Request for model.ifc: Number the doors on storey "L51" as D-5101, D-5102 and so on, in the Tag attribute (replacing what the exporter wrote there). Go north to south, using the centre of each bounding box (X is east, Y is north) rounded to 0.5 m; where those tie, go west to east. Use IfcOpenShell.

First a look at what the model holds.

```python
import ifcopenshell
import ifcopenshell.util.element
import ifcopenshell.util.placement

model = ifcopenshell.open("model.ifc")
print(model.schema)
storey = next(s for s in model.by_type("IfcBuildingStorey") if s.Name == "L51")
doors = [e for e in ifcopenshell.util.element.get_decomposition(storey) if e.is_a("IfcDoor")]
for e in sorted(doors, key=lambda e: e.id()):
    origin = ifcopenshell.util.placement.get_local_placement(e.ObjectPlacement)[:3, 3]
    print(e.id(), e.Tag, e.Name, origin.round(2) + 0.0, sep=" | ")
```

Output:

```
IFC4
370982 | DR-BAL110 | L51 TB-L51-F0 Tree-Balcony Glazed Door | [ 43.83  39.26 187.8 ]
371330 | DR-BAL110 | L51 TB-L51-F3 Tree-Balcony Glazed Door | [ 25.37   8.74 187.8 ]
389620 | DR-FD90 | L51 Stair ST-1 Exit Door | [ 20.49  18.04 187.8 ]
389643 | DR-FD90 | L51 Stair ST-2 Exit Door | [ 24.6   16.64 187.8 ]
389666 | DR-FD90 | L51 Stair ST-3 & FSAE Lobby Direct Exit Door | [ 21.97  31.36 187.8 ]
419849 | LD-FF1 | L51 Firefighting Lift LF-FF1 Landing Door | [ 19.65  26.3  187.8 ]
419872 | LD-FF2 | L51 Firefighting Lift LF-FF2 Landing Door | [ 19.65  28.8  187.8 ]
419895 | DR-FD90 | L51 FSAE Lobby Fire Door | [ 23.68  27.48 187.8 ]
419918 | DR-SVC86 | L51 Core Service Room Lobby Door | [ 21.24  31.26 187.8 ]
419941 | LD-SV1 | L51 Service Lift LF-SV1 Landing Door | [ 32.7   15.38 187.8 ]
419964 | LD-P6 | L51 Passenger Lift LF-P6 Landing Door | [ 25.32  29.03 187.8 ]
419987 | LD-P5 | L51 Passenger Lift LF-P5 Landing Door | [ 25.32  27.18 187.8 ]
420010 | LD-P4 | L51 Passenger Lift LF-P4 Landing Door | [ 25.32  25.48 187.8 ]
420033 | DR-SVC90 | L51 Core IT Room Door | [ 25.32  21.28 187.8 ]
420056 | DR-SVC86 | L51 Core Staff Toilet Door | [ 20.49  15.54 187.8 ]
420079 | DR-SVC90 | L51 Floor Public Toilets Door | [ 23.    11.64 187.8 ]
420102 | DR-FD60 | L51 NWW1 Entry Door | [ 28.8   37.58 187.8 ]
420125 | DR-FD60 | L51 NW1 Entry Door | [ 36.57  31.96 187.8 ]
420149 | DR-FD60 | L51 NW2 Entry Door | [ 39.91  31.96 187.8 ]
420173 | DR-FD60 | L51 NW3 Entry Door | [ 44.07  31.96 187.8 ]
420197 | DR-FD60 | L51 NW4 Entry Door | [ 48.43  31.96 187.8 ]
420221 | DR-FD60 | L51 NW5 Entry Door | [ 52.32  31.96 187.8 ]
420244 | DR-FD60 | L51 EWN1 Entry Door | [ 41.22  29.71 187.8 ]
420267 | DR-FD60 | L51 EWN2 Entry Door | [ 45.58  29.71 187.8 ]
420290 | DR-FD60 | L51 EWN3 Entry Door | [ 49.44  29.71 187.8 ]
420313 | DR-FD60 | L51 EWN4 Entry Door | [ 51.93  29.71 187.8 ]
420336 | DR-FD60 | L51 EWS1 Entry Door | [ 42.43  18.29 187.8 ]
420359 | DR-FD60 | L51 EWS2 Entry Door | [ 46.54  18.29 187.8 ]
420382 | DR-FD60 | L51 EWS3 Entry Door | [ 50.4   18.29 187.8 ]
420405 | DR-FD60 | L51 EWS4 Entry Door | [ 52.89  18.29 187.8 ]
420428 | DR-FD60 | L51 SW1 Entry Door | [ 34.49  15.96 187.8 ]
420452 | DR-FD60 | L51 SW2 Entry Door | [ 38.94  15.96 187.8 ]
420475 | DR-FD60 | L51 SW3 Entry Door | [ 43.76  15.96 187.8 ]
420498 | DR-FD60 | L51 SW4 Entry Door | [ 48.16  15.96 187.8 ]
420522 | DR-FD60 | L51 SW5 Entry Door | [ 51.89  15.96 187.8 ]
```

```python
import ifcopenshell
import ifcopenshell.geom
import ifcopenshell.util.element
import ifcopenshell.util.shape

model = ifcopenshell.open("model.ifc")
settings = ifcopenshell.geom.settings()
settings.set("use-world-coords", True)


def centre(element):
    shape = ifcopenshell.geom.create_shape(settings, element)
    return ifcopenshell.util.shape.get_bbox_centroid(shape.geometry)


storey = next(s for s in model.by_type("IfcBuildingStorey") if s.Name == "L51")
doors = [e for e in ifcopenshell.util.element.get_decomposition(storey) if e.is_a("IfcDoor")]

# Insertion points can sit at a corner or the storey origin, so sort by the geometry (in metres).
centres = {e: centre(e) for e in doors}
doors.sort(key=lambda e: (-round(centres[e][1] / 0.5), centres[e][0]))

for i, e in enumerate(doors, start=1):
    number = f"D-51{i:02d}"
    e.Tag = number
    print(e.id(), number)

model.write("model-out.ifc")
```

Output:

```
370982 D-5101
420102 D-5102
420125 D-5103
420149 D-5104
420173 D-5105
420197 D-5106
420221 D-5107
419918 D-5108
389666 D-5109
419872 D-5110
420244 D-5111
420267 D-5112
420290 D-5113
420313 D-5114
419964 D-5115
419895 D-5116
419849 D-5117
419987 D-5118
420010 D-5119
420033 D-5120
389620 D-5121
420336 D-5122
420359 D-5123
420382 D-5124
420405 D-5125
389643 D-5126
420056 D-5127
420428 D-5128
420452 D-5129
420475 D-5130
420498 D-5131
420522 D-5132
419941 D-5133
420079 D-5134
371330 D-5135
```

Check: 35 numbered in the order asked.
